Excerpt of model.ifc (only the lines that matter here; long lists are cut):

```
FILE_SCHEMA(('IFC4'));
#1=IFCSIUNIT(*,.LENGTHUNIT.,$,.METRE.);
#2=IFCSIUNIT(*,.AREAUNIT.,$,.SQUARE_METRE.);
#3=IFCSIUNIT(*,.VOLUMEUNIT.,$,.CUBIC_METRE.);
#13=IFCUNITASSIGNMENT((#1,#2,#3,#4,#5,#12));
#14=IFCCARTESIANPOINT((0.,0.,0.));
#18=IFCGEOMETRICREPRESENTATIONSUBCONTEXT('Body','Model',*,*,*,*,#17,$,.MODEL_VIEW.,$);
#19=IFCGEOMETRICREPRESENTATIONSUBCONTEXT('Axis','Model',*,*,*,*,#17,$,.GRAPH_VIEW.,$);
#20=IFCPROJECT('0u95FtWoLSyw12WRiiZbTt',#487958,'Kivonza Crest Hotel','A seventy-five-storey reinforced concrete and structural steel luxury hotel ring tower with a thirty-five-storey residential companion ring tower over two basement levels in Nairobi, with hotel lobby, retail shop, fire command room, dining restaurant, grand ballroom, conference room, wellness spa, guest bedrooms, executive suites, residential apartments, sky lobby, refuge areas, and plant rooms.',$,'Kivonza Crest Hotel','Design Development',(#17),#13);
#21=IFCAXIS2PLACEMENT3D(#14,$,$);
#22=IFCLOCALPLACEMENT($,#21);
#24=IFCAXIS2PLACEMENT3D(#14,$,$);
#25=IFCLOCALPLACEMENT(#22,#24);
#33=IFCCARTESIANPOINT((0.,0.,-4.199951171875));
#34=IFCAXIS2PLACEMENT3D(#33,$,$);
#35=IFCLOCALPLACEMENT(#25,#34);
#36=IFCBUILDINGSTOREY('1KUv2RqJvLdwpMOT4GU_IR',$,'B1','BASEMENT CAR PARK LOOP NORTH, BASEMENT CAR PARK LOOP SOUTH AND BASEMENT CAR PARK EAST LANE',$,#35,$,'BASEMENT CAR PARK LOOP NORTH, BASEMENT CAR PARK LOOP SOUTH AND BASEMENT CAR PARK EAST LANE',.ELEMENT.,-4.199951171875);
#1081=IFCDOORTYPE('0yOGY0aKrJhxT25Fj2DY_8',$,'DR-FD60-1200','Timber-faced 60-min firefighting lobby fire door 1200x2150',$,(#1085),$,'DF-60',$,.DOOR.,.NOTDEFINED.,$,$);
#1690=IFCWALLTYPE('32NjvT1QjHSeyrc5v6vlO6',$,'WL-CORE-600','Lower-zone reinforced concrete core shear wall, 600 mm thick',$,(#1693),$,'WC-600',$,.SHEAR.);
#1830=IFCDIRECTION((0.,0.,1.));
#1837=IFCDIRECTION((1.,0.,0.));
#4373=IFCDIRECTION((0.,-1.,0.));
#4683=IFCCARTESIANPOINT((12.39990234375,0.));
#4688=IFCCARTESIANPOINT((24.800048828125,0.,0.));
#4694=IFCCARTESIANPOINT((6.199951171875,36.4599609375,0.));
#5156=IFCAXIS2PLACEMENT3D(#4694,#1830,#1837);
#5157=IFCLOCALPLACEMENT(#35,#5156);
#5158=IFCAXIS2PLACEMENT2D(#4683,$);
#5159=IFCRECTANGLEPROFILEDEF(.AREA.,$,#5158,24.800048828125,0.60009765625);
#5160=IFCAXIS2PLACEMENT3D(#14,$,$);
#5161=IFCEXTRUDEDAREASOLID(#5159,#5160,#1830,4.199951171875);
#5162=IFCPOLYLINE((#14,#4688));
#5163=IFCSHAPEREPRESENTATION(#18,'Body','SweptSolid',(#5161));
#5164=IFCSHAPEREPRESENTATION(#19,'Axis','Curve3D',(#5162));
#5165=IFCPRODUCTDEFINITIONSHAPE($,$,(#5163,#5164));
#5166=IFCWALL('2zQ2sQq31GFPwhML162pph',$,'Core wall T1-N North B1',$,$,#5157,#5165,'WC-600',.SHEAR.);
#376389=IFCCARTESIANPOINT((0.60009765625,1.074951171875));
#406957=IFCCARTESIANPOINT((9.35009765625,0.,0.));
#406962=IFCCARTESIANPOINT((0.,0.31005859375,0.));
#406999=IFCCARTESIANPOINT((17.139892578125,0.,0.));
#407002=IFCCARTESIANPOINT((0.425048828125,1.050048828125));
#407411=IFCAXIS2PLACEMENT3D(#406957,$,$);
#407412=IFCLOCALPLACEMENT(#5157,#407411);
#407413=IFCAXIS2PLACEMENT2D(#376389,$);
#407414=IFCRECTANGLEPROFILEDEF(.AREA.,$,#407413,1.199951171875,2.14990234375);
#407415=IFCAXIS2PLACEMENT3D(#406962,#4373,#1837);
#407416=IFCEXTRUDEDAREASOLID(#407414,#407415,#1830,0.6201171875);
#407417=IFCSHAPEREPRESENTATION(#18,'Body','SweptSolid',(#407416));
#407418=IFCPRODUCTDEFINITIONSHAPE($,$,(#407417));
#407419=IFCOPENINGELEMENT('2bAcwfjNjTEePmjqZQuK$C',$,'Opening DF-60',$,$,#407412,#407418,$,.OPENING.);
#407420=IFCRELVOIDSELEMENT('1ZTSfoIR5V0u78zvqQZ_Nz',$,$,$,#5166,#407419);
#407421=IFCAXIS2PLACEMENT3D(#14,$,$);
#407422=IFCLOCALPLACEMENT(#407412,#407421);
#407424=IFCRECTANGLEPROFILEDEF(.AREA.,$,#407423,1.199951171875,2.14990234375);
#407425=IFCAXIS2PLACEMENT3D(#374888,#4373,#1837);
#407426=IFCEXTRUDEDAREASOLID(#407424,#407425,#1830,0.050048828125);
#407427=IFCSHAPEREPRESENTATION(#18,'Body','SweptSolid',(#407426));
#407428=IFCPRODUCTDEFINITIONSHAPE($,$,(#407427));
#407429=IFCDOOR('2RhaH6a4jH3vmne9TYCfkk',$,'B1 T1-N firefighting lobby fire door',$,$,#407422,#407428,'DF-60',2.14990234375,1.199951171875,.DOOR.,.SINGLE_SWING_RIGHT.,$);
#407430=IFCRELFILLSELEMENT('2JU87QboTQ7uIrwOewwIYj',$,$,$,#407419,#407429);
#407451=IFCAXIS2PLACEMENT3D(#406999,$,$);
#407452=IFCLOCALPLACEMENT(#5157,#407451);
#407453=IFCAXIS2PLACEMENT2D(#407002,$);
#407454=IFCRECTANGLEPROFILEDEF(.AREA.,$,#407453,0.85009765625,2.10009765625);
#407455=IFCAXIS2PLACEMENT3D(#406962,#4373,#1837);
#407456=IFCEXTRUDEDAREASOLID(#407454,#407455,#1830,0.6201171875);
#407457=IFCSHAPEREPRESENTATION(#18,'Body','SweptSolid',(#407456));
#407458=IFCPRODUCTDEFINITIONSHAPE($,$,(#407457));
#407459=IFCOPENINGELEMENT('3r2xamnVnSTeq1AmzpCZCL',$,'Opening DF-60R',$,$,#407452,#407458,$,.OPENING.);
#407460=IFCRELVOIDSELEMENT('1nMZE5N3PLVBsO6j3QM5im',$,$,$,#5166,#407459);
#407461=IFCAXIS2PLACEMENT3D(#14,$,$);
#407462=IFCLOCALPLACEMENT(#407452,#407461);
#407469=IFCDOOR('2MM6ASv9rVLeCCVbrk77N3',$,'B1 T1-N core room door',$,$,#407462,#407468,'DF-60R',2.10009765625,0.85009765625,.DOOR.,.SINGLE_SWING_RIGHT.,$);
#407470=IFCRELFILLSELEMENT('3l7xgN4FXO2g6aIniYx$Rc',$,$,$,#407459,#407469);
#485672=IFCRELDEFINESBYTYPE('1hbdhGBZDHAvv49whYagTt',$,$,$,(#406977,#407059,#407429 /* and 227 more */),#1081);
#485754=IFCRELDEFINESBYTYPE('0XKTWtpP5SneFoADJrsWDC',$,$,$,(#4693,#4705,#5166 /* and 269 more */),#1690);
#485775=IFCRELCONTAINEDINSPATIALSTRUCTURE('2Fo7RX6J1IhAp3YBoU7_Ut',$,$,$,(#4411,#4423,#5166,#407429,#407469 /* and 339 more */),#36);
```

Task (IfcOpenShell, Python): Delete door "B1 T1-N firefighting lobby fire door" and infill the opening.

```python
import ifcopenshell
import ifcopenshell.api.feature
import ifcopenshell.api.root
import ifcopenshell.geom
import ifcopenshell.util.shape

model = ifcopenshell.open("model.ifc")
settings = ifcopenshell.geom.settings()


def volume(element):
    """Net volume in cubic metres, openings subtracted."""
    shape = ifcopenshell.geom.create_shape(settings, element)
    return ifcopenshell.util.shape.get_volume(shape.geometry)


door = model.by_guid("2RhaH6a4jH3vmne9TYCfkk")
opening = door.FillsVoids[0].RelatingOpeningElement
wall = opening.VoidsElements[0].RelatingBuildingElement
before = volume(wall)

ifcopenshell.api.root.remove_product(model, product=door)
ifcopenshell.api.feature.remove_feature(model, feature=opening)

after = volume(wall)

print(f"wall volume {before:.3f} -> {after:.3f} m3")

model.write("model_edited.ifc")
```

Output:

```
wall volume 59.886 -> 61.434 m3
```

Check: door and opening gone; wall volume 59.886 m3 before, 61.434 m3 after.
